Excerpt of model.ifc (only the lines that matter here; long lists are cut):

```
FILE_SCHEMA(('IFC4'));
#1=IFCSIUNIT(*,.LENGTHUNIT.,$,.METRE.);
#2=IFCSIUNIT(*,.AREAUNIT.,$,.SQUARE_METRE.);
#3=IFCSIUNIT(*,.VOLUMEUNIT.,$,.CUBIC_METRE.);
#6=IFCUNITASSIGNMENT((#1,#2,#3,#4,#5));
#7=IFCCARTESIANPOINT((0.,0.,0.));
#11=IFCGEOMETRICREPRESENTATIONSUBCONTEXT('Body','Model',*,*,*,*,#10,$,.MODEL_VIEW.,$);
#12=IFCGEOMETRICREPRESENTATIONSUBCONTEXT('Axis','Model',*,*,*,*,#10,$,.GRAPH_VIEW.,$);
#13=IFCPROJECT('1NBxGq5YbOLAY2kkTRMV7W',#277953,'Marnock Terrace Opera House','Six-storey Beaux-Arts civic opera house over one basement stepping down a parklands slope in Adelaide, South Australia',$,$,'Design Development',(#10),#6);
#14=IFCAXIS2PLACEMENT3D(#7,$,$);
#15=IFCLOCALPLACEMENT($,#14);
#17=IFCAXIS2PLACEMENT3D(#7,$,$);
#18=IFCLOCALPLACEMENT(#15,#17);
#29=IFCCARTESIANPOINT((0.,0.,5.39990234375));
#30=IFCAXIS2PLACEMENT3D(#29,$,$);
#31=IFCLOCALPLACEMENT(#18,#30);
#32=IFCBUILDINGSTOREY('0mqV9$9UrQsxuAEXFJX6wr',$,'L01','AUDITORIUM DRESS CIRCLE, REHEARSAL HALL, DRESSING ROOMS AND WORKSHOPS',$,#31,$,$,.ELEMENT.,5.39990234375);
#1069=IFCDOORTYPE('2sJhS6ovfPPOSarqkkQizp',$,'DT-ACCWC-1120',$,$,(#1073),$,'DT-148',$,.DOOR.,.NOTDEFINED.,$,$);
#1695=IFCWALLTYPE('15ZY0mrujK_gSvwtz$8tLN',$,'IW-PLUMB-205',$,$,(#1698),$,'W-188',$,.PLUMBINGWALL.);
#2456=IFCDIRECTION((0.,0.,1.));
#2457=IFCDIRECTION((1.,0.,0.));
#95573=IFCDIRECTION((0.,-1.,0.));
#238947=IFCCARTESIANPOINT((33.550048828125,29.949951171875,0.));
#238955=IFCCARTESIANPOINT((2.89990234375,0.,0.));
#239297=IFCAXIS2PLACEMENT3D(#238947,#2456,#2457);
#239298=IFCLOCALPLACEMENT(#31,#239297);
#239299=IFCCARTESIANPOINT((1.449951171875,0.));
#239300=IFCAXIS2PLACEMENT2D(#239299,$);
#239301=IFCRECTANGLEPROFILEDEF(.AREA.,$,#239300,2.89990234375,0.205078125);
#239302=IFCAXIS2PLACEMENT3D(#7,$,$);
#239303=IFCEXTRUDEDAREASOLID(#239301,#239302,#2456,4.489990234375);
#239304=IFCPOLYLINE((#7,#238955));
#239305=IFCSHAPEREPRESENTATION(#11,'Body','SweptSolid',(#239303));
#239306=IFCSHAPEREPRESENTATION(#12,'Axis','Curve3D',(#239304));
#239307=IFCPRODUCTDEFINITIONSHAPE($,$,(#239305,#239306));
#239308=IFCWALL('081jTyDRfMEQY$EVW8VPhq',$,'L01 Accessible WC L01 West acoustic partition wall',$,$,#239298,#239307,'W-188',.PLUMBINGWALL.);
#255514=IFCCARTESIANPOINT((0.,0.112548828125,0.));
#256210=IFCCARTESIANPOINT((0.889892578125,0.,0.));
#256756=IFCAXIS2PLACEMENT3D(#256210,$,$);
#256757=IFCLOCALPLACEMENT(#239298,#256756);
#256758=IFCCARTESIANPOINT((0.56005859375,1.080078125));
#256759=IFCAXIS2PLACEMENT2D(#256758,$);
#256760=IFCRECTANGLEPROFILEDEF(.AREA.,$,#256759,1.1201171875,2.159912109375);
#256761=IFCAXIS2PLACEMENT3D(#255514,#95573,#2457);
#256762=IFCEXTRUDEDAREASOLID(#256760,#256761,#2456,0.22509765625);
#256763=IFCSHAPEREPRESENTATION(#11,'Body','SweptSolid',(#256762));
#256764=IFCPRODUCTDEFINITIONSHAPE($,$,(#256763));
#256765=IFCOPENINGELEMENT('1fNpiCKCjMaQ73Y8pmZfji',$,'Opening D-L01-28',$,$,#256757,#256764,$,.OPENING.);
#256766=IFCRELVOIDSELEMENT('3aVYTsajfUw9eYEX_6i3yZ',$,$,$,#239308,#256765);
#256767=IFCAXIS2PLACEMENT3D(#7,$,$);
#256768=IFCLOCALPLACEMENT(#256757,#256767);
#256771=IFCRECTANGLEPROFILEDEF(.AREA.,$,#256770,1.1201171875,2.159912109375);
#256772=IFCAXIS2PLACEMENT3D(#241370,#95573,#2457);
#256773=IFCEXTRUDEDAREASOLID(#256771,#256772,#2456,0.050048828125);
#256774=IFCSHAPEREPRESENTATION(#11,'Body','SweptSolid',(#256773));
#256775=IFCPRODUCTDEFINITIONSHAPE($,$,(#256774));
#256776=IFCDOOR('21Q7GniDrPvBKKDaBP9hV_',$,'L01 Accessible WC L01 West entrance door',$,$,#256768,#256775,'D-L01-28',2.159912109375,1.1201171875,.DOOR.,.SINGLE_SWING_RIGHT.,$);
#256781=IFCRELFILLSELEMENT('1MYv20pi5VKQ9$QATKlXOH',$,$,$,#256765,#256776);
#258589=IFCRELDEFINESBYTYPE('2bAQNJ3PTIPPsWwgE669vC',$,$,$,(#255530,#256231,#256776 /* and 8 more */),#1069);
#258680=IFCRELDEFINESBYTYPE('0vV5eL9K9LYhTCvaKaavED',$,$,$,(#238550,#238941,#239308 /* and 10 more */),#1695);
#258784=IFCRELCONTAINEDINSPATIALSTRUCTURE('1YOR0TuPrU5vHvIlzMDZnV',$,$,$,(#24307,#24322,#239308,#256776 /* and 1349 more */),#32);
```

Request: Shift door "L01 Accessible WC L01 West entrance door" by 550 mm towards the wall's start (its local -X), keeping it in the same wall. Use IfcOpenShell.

```python
import ifcopenshell
import ifcopenshell.api.geometry
import ifcopenshell.util.placement
import ifcopenshell.util.unit

model = ifcopenshell.open("model.ifc")
unit_scale = ifcopenshell.util.unit.calculate_unit_scale(model)

door = model.by_guid("21Q7GniDrPvBKKDaBP9hV_")
opening = door.FillsVoids[0].RelatingOpeningElement
wall = opening.VoidsElements[0].RelatingBuildingElement

wall_matrix = ifcopenshell.util.placement.get_local_placement(wall.ObjectPlacement)
shift = wall_matrix[:3, 0] * -0.55 / unit_scale
before = ifcopenshell.util.placement.get_local_placement(door.ObjectPlacement)[:3, 3].copy()

# The door is placed relative to its opening, so it follows when the opening moves.
matrix = ifcopenshell.util.placement.get_local_placement(opening.ObjectPlacement)
matrix[:3, 3] += shift
ifcopenshell.api.geometry.edit_object_placement(
    model, product=opening, matrix=matrix, is_si=False, should_transform_children=True
)

after = ifcopenshell.util.placement.get_local_placement(door.ObjectPlacement)[:3, 3]
print("door moved by", (after - before).round(3) + 0.0)

model.write("model_edited.ifc")
```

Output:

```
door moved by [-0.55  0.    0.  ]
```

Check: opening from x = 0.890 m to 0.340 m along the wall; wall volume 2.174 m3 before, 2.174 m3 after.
